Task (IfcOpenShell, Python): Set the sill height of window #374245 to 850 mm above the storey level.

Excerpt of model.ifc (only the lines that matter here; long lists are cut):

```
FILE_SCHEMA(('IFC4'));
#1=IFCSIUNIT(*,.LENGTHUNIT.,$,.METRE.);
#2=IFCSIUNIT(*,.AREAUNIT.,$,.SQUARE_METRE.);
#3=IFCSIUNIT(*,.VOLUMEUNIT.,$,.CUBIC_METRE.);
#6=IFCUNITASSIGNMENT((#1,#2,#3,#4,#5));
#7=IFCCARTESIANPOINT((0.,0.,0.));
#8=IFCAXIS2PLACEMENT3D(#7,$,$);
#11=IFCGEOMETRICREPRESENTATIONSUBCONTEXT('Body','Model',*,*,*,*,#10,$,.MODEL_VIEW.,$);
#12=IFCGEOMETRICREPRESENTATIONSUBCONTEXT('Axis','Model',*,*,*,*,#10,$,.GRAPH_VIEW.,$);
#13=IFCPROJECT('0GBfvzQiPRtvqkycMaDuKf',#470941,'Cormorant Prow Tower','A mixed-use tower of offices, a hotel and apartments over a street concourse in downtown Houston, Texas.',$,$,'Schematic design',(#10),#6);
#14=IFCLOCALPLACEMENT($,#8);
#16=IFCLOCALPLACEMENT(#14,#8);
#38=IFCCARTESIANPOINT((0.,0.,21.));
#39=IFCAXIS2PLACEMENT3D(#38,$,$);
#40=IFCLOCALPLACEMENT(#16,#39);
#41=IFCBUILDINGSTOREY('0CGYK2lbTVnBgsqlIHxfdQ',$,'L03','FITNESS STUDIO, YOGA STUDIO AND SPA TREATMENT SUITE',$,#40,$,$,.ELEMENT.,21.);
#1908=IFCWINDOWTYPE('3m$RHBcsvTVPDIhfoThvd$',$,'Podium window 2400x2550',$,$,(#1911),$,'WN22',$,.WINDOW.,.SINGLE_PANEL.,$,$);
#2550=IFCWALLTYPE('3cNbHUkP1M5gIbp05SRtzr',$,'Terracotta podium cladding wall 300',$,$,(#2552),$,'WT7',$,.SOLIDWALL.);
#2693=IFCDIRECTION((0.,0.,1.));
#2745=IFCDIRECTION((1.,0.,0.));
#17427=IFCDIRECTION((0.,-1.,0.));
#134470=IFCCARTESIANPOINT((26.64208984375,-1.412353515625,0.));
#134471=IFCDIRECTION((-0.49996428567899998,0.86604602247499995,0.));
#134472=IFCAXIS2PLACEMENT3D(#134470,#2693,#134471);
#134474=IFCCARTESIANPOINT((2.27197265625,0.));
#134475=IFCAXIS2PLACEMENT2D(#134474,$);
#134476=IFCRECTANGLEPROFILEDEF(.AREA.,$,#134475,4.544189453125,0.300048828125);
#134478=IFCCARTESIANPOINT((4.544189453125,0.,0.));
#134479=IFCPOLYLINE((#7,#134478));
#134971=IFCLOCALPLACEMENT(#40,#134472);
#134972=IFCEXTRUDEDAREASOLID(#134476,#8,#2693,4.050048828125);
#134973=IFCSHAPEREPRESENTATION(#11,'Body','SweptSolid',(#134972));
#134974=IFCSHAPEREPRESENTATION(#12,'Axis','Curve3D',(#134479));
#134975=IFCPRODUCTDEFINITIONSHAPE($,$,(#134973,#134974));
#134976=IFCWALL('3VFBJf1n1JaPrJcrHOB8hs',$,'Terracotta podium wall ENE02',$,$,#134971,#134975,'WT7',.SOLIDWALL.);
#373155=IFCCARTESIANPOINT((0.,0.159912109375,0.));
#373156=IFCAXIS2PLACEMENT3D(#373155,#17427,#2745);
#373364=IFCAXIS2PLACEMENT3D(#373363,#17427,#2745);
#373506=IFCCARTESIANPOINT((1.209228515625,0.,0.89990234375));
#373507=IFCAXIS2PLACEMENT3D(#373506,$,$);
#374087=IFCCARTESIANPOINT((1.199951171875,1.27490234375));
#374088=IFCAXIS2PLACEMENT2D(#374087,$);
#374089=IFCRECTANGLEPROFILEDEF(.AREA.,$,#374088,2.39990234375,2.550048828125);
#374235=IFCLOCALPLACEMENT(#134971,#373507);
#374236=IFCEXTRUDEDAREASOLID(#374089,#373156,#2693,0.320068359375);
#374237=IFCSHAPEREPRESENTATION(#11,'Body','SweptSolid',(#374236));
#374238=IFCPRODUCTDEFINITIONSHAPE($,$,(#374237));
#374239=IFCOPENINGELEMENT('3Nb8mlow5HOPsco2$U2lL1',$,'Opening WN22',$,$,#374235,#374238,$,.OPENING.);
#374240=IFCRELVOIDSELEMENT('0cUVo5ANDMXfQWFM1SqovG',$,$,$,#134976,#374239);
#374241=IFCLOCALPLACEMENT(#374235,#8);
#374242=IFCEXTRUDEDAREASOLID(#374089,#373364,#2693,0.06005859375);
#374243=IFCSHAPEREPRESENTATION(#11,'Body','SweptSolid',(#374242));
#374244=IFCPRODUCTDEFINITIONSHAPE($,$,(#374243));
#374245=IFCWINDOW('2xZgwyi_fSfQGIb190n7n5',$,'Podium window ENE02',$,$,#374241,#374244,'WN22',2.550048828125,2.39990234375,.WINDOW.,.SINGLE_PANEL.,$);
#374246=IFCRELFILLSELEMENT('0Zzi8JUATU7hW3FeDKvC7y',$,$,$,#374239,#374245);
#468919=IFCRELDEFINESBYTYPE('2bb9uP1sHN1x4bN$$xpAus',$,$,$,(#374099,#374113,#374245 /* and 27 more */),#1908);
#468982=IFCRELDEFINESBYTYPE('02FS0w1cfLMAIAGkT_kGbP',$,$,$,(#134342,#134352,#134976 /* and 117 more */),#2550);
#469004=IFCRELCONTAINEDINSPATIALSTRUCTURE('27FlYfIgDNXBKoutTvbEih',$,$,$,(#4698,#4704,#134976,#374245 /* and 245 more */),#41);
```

```python
import numpy as np
import ifcopenshell
import ifcopenshell.api.geometry
import ifcopenshell.geom
import ifcopenshell.util.element
import ifcopenshell.util.placement
import ifcopenshell.util.shape
import ifcopenshell.util.unit

model = ifcopenshell.open("model.ifc")
unit_scale = ifcopenshell.util.unit.calculate_unit_scale(model)

window = model.by_id(374245)
opening = window.FillsVoids[0].RelatingOpeningElement
storey = ifcopenshell.util.element.get_container(window, ifc_class="IfcBuildingStorey")
level = ifcopenshell.util.placement.get_local_placement(storey.ObjectPlacement)[2, 3]

# The opening's origin need not be at the sill, so measure its lowest point.
shape = ifcopenshell.geom.create_shape(ifcopenshell.geom.settings(), opening)
bottom = ifcopenshell.util.shape.get_shape_bottom_elevation(shape, shape.geometry) / unit_scale
dz = level + 0.85 - bottom

shift = np.array([0.0, 0.0, dz])
# The window is placed relative to its opening, so it follows when the opening moves.
matrix = ifcopenshell.util.placement.get_local_placement(opening.ObjectPlacement)
matrix[:3, 3] += shift
ifcopenshell.api.geometry.edit_object_placement(
    model, product=opening, matrix=matrix, is_si=False, should_transform_children=True
)

print(f"moved by {dz * unit_scale:+.3f} m")

model.write("model_updated.ifc")
```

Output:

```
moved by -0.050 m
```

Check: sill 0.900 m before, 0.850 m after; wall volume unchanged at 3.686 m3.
